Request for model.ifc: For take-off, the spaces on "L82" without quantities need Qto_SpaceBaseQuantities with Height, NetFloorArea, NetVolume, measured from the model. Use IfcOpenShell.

First a look at what the model holds.

```python
import ifcopenshell
import ifcopenshell.util.element
import ifcopenshell.util.unit

model = ifcopenshell.open("model.ifc")
print(model.schema)
for unit_type in ("LENGTHUNIT", "AREAUNIT", "VOLUMEUNIT"):
    print(unit_type, ifcopenshell.util.unit.calculate_unit_scale(model, unit_type))
storey = next(s for s in model.by_type("IfcBuildingStorey") if s.Name == "L82")
spaces = [e for e in ifcopenshell.util.element.get_decomposition(storey) if e.is_a("IfcSpace")]
for e in sorted(spaces, key=lambda e: e.id()):
    print(e.id(), e.is_a(), e.Name, list(ifcopenshell.util.element.get_psets(e, qtos_only=True)), sep=" | ")
```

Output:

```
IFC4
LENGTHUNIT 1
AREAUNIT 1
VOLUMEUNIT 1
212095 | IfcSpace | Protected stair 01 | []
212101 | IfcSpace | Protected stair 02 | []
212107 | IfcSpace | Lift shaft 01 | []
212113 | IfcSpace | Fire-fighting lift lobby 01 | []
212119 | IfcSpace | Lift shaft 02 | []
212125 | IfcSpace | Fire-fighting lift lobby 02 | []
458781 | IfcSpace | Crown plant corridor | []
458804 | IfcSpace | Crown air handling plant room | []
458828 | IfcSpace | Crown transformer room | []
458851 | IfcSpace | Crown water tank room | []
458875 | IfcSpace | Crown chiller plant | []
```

```python
import ifcopenshell
import ifcopenshell.api.pset
import ifcopenshell.geom
import ifcopenshell.util.element
import ifcopenshell.util.shape
import ifcopenshell.util.unit

model = ifcopenshell.open("model.ifc")
unit_scale = ifcopenshell.util.unit.calculate_unit_scale(model)
area_scale = ifcopenshell.util.unit.calculate_unit_scale(model, "AREAUNIT")
volume_scale = ifcopenshell.util.unit.calculate_unit_scale(model, "VOLUMEUNIT")
settings = ifcopenshell.geom.settings()

storey = next(s for s in model.by_type("IfcBuildingStorey") if s.Name == "L82")
spaces = [e for e in ifcopenshell.util.element.get_decomposition(storey) if e.is_a("IfcSpace")]

for e in sorted(spaces, key=lambda e: e.id()):
    if ifcopenshell.util.element.get_psets(e, qtos_only=True, should_inherit=False):
        continue
    # Geometry comes back in metres, in the element's own axes.
    shape = ifcopenshell.geom.create_shape(settings, e)
    values = {
        "Height": ifcopenshell.util.shape.get_z(shape.geometry) / unit_scale,
        "NetFloorArea": ifcopenshell.util.shape.get_footprint_area(shape.geometry) / area_scale,
        "NetVolume": ifcopenshell.util.shape.get_volume(shape.geometry) / volume_scale,
    }
    qto = ifcopenshell.api.pset.add_qto(model, product=e, name="Qto_SpaceBaseQuantities")
    ifcopenshell.api.pset.edit_qto(model, qto=qto, properties=values)
    print(e.id(), {k: round(v, 3) for k, v in values.items()})

model.write("model_rev.ifc")
```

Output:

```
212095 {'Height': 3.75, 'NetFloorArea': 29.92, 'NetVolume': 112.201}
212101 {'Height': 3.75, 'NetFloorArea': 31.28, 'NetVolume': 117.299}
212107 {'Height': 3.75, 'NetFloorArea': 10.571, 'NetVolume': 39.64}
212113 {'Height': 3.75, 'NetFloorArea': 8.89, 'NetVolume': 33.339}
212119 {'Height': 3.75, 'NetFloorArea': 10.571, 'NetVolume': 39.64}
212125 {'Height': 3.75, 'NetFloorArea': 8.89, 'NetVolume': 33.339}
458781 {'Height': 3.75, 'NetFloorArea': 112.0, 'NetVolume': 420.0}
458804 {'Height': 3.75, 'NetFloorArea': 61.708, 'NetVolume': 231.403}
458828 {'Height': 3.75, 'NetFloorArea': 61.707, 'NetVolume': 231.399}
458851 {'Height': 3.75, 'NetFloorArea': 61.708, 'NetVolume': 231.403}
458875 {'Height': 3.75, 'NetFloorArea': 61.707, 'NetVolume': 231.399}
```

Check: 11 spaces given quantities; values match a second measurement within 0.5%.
